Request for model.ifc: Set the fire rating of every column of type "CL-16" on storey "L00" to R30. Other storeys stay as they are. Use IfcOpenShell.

First a look at what the model holds.

```python
import ifcopenshell
import ifcopenshell.util.element

model = ifcopenshell.open("model.ifc")
print(model.schema)
storey = next(s for s in model.by_type("IfcBuildingStorey") if s.Name == "L00")
columns = [e for e in ifcopenshell.util.element.get_decomposition(storey) if e.is_a("IfcColumn")]
seen = {}
for e in columns:
    element_type = ifcopenshell.util.element.get_type(e)
    key = (element_type.Name if element_type != e and element_type else None, ifcopenshell.util.element.get_pset(e, "Pset_ColumnCommon", "FireRating"))
    seen[key] = seen.get(key, 0) + 1
for (name, value), count in sorted(seen.items(), key=str):
    print(count, "x", name, "|", value)
```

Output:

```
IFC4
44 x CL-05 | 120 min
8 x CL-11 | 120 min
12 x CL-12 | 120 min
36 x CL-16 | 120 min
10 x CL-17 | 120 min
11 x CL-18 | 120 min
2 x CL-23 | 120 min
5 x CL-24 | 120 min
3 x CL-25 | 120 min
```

```python
import ifcopenshell
import ifcopenshell.api.pset
import ifcopenshell.util.element

model = ifcopenshell.open("model.ifc")

storey = next(s for s in model.by_type("IfcBuildingStorey") if s.Name == "L00")
columns = [e for e in ifcopenshell.util.element.get_decomposition(storey) if e.is_a("IfcColumn")]

count = 0
for e in columns:
    element_type = ifcopenshell.util.element.get_type(e)
    if element_type in (None, e) or element_type.Name != "CL-16":
        continue
    # add_pset returns the element's existing set when there is one.
    pset = ifcopenshell.api.pset.add_pset(model, product=e, name="Pset_ColumnCommon")
    ifcopenshell.api.pset.edit_pset(model, pset=pset, properties={"FireRating": "R30"})
    count += 1

print(count, "columns updated")

model.write("model_updated.ifc")
```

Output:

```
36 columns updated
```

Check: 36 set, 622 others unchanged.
